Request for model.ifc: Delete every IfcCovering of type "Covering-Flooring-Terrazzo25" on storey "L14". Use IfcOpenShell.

First a look at what the model holds.

```python
import ifcopenshell
import ifcopenshell.util.element

model = ifcopenshell.open("model.ifc")
print(model.schema)
storey = next(s for s in model.by_type("IfcBuildingStorey") if s.Name == "L14")
coverings = [e for e in ifcopenshell.util.element.get_decomposition(storey) if e.is_a("IfcCovering")]
seen = {}
for e in coverings:
    element_type = ifcopenshell.util.element.get_type(e)
    name = element_type.Name if element_type not in (None, e) else None
    seen[name] = seen.get(name, 0) + 1
for name, count in sorted(seen.items(), key=str):
    print(count, "x", name)
```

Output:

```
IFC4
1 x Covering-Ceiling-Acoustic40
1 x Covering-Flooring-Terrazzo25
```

```python
import ifcopenshell
import ifcopenshell.api.root
import ifcopenshell.util.element

model = ifcopenshell.open("model.ifc")

storey = next(s for s in model.by_type("IfcBuildingStorey") if s.Name == "L14")
coverings = [e for e in ifcopenshell.util.element.get_decomposition(storey) if e.is_a("IfcCovering")]
targets = [e for e in coverings if (t := ifcopenshell.util.element.get_type(e)) not in (None, e) and t.Name == "Covering-Flooring-Terrazzo25"]

for e in targets:
    ifcopenshell.api.root.remove_product(model, product=e)
print(len(targets), "removed")

model.write("model_rev.ifc")
```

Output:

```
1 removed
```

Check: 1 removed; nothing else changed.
